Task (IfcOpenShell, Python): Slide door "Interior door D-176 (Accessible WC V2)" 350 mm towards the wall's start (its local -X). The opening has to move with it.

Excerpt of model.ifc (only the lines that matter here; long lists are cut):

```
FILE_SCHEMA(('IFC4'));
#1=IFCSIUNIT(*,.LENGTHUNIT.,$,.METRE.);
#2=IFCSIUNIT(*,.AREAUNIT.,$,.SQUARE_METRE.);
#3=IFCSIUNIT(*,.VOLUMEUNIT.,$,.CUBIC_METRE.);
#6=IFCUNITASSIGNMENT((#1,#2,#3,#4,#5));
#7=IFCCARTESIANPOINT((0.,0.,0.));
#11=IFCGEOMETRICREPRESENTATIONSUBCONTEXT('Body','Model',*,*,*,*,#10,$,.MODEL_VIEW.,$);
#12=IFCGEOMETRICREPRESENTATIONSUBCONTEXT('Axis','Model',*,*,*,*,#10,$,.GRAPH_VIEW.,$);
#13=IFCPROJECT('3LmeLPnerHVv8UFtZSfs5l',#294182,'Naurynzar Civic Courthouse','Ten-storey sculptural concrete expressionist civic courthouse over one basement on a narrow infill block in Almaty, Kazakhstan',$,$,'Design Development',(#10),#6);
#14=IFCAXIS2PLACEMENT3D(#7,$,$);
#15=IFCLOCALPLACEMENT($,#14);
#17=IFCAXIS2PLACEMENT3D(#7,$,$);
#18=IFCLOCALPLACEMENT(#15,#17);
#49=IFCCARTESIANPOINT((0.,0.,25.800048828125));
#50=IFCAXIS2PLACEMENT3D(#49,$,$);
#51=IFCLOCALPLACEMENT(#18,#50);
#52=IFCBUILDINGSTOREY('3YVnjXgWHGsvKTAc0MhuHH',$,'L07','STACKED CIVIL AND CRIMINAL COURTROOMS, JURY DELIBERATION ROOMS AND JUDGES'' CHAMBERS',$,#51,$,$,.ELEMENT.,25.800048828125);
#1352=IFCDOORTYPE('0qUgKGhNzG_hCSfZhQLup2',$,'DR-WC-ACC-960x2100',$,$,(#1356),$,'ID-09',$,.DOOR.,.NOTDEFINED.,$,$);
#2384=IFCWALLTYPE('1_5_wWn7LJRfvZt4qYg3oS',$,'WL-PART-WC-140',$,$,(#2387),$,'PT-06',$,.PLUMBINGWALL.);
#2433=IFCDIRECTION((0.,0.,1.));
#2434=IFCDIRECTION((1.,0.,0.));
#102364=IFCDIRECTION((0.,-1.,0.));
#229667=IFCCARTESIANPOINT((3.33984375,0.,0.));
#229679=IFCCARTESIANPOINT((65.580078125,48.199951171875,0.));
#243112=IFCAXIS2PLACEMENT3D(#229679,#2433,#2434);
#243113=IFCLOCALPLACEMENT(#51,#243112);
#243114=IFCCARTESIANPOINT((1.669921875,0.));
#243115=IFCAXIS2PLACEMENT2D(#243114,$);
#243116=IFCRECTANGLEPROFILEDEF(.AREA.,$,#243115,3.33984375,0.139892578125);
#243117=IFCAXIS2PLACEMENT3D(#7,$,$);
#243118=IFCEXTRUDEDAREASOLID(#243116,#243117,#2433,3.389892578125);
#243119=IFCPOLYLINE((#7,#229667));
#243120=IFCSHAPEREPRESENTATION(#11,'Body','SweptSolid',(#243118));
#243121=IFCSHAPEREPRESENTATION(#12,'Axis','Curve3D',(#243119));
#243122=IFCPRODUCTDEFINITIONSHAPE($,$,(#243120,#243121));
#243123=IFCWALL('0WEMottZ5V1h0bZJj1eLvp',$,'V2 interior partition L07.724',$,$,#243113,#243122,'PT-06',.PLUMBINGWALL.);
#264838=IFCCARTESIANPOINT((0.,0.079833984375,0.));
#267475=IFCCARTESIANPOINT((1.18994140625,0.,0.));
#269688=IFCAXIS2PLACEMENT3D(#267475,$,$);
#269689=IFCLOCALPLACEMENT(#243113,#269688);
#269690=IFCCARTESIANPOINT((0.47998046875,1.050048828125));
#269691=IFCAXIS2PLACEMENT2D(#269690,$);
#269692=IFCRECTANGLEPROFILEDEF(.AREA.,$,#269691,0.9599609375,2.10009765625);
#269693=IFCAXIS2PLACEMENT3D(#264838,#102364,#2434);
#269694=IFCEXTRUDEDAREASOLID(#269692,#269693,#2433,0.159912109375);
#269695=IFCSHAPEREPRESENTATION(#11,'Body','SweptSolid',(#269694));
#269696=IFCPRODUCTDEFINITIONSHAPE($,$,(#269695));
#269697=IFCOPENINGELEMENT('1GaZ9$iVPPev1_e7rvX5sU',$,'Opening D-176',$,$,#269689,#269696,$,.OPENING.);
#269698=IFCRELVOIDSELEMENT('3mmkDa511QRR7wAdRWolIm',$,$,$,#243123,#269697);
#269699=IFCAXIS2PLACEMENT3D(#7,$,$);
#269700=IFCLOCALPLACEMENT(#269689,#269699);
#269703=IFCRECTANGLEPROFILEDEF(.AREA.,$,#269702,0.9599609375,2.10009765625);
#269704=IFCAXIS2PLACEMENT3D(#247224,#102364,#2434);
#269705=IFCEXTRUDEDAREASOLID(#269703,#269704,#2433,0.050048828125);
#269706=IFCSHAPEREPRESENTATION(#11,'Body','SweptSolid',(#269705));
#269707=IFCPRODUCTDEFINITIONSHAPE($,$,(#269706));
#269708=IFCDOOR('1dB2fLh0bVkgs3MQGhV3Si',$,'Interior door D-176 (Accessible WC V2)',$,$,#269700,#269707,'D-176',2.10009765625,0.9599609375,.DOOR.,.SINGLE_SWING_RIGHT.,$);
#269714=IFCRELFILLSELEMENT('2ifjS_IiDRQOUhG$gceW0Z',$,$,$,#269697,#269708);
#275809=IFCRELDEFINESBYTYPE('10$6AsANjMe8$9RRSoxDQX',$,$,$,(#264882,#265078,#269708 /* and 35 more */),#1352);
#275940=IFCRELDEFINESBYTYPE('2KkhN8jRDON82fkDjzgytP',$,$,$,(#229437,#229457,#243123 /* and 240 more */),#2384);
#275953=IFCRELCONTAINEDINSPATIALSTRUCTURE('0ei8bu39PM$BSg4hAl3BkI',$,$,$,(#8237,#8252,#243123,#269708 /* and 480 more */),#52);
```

```python
import ifcopenshell
import ifcopenshell.api.geometry
import ifcopenshell.util.placement

model = ifcopenshell.open("model.ifc")

door = model.by_id(269708)
opening = door.FillsVoids[0].RelatingOpeningElement
wall = opening.VoidsElements[0].RelatingBuildingElement

wall_matrix = ifcopenshell.util.placement.get_local_placement(wall.ObjectPlacement)
shift = wall_matrix[:3, 0] * -0.35
before = ifcopenshell.util.placement.get_local_placement(door.ObjectPlacement)[:3, 3].copy()

# The door is placed relative to its opening, so it follows when the opening moves.
matrix = ifcopenshell.util.placement.get_local_placement(opening.ObjectPlacement)
matrix[:3, 3] += shift
ifcopenshell.api.geometry.edit_object_placement(
    model, product=opening, matrix=matrix, is_si=False, should_transform_children=True
)

after = ifcopenshell.util.placement.get_local_placement(door.ObjectPlacement)[:3, 3]
print("door moved by", (after - before).round(3) + 0.0)

model.write("model-out.ifc")
```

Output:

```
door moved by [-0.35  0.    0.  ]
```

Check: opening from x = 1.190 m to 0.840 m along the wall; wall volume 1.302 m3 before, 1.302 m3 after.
